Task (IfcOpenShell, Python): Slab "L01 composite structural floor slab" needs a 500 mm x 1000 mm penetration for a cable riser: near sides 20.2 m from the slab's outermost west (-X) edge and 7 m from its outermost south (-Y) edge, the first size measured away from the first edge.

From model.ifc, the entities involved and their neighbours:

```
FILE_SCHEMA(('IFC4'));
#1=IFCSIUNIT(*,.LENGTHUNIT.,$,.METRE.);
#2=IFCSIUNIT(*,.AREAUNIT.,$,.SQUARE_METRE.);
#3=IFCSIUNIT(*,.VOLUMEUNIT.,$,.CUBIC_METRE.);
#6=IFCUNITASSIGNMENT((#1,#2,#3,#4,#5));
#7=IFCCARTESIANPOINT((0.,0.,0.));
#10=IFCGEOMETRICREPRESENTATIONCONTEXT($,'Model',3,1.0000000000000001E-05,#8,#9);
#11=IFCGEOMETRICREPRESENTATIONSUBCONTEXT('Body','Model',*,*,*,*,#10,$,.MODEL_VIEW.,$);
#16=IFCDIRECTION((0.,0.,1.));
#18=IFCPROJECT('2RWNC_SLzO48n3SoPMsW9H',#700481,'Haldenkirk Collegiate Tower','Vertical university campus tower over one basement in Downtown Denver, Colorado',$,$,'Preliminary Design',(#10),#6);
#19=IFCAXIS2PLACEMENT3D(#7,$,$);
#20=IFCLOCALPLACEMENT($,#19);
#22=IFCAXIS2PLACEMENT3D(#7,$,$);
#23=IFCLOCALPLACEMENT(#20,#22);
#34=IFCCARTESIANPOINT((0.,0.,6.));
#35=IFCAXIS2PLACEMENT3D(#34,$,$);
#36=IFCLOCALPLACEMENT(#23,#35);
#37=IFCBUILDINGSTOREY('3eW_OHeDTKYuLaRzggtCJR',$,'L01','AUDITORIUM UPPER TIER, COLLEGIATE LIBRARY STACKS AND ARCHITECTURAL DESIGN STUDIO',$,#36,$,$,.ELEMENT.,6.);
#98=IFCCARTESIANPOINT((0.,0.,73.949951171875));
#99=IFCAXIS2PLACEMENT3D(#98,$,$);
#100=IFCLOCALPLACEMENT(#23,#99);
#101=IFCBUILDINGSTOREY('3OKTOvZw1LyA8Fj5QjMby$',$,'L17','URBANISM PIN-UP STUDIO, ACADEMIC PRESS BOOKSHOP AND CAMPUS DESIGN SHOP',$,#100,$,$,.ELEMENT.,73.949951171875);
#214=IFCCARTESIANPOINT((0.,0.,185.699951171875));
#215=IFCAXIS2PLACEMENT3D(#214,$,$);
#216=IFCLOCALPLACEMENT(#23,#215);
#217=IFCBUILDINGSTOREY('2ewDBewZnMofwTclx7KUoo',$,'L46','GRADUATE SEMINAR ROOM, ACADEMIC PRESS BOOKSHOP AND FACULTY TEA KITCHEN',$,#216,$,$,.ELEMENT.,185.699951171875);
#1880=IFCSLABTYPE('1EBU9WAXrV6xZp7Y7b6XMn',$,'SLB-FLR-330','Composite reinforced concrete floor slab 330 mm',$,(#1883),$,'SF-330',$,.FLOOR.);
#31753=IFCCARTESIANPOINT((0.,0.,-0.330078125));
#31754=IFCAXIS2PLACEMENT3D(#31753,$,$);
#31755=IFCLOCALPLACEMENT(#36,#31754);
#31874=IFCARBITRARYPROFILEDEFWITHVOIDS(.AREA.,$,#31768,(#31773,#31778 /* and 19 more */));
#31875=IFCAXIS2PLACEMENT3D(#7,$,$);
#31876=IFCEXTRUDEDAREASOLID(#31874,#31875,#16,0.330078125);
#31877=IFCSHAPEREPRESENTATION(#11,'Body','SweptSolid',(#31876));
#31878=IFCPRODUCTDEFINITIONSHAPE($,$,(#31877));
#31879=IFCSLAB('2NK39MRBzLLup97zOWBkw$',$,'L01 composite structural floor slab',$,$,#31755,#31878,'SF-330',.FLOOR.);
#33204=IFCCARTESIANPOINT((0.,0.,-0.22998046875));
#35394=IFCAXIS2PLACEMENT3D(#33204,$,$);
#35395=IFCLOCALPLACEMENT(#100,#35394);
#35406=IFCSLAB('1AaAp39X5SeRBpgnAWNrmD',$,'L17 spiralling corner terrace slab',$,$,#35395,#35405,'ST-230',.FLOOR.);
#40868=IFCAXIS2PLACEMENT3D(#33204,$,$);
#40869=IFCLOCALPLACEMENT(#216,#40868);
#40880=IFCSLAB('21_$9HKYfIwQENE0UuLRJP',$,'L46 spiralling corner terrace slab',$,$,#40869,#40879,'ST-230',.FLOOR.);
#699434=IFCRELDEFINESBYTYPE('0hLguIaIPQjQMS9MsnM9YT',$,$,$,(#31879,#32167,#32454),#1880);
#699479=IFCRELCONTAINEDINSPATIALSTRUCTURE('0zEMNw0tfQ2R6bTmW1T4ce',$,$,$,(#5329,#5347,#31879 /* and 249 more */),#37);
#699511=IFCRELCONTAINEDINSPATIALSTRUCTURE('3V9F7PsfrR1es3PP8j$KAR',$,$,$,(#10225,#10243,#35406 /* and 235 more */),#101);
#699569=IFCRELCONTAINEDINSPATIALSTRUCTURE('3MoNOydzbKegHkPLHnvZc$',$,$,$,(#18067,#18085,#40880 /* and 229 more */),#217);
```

```python
import numpy as np
import ifcopenshell
import ifcopenshell.api.feature
import ifcopenshell.api.geometry
import ifcopenshell.api.root
import ifcopenshell.geom
import ifcopenshell.util.placement
import ifcopenshell.util.representation
import ifcopenshell.util.shape
import ifcopenshell.util.unit

model = ifcopenshell.open("model.ifc")
unit_scale = ifcopenshell.util.unit.calculate_unit_scale(model)
settings = ifcopenshell.geom.settings()


def volume(element):
    """Net volume in cubic metres, openings subtracted."""
    shape = ifcopenshell.geom.create_shape(settings, element)
    return ifcopenshell.util.shape.get_volume(shape.geometry)


slab = model.by_id(31879)
before = volume(slab)

# Extent in the slab's own axes, in metres. The edges named are its -X and -Y sides.
slab_shape = ifcopenshell.geom.create_shape(settings, slab)
vertices = ifcopenshell.util.shape.get_vertices(slab_shape.geometry)
x_min, y_min, bottom = vertices.min(axis=0)
top = vertices[:, 2].max()

opening = ifcopenshell.api.root.create_entity(model, ifc_class="IfcOpeningElement", name="Cable riser opening", predefined_type="OPENING")
context = ifcopenshell.util.representation.get_context(model, "Model", "Body", "MODEL_VIEW")
width, depth = 0.5, 1
outline = [(0.0, 0.0), (width, 0.0), (width, depth), (0.0, depth), (0.0, 0.0)]
# Overshoot both faces by 50 mm so the cut is clean.
shape = ifcopenshell.api.geometry.add_slab_representation(
    model, context=context, depth=top - bottom + 0.1, polyline=outline
)
ifcopenshell.api.geometry.assign_representation(model, product=opening, representation=shape)

matrix = ifcopenshell.util.placement.get_local_placement(slab.ObjectPlacement)
matrix[:, 3] = matrix @ np.append(np.array([x_min + 20.2, y_min + 7, bottom - 0.05]) / unit_scale, 1.0)
ifcopenshell.api.geometry.edit_object_placement(model, product=opening, matrix=matrix, is_si=False)
ifcopenshell.api.feature.add_feature(model, feature=opening, element=slab)

after = volume(slab)

print(f"slab volume {before:.3f} -> {after:.3f} m3")

model.write("model_edited.ifc")
```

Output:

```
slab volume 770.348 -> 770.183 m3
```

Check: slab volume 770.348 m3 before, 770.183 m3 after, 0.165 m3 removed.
